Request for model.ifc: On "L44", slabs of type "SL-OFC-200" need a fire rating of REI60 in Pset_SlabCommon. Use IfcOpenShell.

First a look at what the model holds.

```python
import ifcopenshell
import ifcopenshell.util.element

model = ifcopenshell.open("model.ifc")
print(model.schema)
storey = next(s for s in model.by_type("IfcBuildingStorey") if s.Name == "L44")
slabs = [e for e in ifcopenshell.util.element.get_decomposition(storey) if e.is_a("IfcSlab")]
seen = {}
for e in slabs:
    element_type = ifcopenshell.util.element.get_type(e)
    key = (element_type.Name if element_type != e and element_type else None, ifcopenshell.util.element.get_pset(e, "Pset_SlabCommon", "FireRating"))
    seen[key] = seen.get(key, 0) + 1
for (name, value), count in sorted(seen.items(), key=str):
    print(count, "x", name, "|", value)
```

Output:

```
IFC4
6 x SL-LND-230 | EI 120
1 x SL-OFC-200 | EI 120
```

```python
import ifcopenshell
import ifcopenshell.api.pset
import ifcopenshell.util.element

model = ifcopenshell.open("model.ifc")

storey = next(s for s in model.by_type("IfcBuildingStorey") if s.Name == "L44")
slabs = [e for e in ifcopenshell.util.element.get_decomposition(storey) if e.is_a("IfcSlab")]

count = 0
for e in slabs:
    element_type = ifcopenshell.util.element.get_type(e)
    if element_type in (None, e) or element_type.Name != "SL-OFC-200":
        continue
    # add_pset returns the element's existing set when there is one.
    pset = ifcopenshell.api.pset.add_pset(model, product=e, name="Pset_SlabCommon")
    ifcopenshell.api.pset.edit_pset(model, pset=pset, properties={"FireRating": "REI60"})
    count += 1

print(count, "slabs updated")

model.write("model_rev.ifc")
```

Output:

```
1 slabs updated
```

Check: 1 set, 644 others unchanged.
